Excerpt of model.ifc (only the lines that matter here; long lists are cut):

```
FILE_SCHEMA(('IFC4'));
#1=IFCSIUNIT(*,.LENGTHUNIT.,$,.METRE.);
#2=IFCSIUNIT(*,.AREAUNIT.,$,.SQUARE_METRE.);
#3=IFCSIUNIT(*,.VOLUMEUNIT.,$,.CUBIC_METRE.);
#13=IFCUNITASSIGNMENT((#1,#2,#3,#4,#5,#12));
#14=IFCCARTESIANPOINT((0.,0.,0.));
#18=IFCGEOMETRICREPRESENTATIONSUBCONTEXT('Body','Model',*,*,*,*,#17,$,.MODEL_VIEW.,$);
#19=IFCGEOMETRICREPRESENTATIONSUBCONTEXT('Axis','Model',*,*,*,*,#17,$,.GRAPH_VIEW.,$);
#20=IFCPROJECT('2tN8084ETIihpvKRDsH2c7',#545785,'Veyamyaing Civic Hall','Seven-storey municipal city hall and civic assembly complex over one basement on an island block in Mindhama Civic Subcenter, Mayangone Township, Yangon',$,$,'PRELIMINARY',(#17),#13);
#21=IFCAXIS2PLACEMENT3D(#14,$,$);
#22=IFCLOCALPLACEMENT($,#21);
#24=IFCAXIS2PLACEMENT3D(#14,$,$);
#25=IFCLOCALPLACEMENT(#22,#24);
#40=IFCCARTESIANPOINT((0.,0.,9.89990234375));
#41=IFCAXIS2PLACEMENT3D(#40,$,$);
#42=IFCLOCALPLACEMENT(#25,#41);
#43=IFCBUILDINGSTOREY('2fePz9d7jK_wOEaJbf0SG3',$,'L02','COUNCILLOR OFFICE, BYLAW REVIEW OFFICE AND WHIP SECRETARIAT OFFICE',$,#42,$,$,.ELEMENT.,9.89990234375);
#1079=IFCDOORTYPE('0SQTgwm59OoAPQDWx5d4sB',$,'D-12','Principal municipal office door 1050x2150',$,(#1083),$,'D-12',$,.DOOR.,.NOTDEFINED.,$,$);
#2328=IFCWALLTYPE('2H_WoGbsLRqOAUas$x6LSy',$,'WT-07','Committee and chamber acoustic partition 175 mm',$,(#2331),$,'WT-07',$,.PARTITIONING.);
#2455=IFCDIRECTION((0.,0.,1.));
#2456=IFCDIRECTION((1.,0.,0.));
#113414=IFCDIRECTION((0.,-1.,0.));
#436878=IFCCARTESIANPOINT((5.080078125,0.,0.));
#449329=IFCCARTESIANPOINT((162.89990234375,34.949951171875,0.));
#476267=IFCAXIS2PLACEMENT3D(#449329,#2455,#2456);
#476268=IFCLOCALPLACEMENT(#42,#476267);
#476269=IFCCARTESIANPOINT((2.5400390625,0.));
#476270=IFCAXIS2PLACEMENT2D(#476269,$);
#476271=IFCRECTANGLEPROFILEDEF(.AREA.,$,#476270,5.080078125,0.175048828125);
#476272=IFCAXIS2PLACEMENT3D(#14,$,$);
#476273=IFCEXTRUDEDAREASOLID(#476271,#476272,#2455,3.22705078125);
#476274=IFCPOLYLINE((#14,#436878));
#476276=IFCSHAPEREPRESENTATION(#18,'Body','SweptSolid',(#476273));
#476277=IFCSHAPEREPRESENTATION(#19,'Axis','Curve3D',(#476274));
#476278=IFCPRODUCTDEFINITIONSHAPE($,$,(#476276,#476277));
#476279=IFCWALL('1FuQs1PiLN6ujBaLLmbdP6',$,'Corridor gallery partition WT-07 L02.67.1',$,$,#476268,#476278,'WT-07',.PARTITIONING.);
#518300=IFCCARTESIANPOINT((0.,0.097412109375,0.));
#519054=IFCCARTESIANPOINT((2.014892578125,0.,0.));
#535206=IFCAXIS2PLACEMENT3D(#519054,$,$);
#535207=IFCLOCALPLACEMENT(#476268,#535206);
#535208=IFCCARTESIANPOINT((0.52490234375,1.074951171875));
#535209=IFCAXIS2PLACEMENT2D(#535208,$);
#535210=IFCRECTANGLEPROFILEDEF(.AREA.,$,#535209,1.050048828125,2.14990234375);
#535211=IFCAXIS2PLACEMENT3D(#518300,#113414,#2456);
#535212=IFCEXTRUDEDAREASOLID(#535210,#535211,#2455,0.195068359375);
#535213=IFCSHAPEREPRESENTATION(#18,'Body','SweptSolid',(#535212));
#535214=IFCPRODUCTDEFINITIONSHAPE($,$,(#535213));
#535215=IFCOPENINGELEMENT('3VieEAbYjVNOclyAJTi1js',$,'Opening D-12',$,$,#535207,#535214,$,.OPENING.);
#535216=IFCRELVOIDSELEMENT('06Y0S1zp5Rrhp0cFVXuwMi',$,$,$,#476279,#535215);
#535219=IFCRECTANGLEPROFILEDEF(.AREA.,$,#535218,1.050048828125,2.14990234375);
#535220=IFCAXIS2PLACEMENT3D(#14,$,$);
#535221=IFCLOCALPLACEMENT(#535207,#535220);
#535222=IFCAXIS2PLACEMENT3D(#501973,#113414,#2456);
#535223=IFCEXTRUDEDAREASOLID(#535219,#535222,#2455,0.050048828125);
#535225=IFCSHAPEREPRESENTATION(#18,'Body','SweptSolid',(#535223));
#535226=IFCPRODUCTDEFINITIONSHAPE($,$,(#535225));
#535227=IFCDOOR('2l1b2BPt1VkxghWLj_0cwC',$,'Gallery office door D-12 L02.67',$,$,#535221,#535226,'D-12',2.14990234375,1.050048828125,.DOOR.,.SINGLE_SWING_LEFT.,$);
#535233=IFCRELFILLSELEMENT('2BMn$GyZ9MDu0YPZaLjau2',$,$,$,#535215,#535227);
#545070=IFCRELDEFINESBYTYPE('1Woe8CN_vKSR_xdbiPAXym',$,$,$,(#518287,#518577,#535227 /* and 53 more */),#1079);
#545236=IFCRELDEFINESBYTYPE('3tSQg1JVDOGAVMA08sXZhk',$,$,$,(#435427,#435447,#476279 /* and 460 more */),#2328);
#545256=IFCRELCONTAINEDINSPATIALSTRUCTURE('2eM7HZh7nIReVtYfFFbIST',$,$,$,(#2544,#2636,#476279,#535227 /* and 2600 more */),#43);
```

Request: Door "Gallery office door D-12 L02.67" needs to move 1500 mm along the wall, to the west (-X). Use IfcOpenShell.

```python
import ifcopenshell
import ifcopenshell.api.geometry
import ifcopenshell.util.placement
import ifcopenshell.util.unit

model = ifcopenshell.open("model.ifc")
unit_scale = ifcopenshell.util.unit.calculate_unit_scale(model)

door = model.by_id(535227)
opening = door.FillsVoids[0].RelatingOpeningElement
wall = opening.VoidsElements[0].RelatingBuildingElement

wall_matrix = ifcopenshell.util.placement.get_local_placement(wall.ObjectPlacement)
shift = wall_matrix[:3, 0] * -1.5 / unit_scale
before = ifcopenshell.util.placement.get_local_placement(door.ObjectPlacement)[:3, 3].copy()

# The door is placed relative to its opening, so it follows when the opening moves.
matrix = ifcopenshell.util.placement.get_local_placement(opening.ObjectPlacement)
matrix[:3, 3] += shift
ifcopenshell.api.geometry.edit_object_placement(
    model, product=opening, matrix=matrix, is_si=False, should_transform_children=True
)

after = ifcopenshell.util.placement.get_local_placement(door.ObjectPlacement)[:3, 3]
print("door moved by", (after - before).round(3) + 0.0)

model.write("model_edited.ifc")
```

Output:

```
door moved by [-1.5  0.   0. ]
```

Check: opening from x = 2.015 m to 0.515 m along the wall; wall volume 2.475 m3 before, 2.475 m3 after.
